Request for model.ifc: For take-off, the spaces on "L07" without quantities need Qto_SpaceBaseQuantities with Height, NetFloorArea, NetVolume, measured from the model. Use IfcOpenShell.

First a look at what the model holds.

```python
import ifcopenshell
import ifcopenshell.util.element
import ifcopenshell.util.unit

model = ifcopenshell.open("model.ifc")
print(model.schema)
for unit_type in ("LENGTHUNIT", "AREAUNIT", "VOLUMEUNIT"):
    print(unit_type, ifcopenshell.util.unit.calculate_unit_scale(model, unit_type))
storey = next(s for s in model.by_type("IfcBuildingStorey") if s.Name == "L07")
spaces = [e for e in ifcopenshell.util.element.get_decomposition(storey) if e.is_a("IfcSpace")]
for e in sorted(spaces, key=lambda e: e.id()):
    print(e.id(), e.is_a(), e.Name, list(ifcopenshell.util.element.get_psets(e, qtos_only=True)), sep=" | ")
```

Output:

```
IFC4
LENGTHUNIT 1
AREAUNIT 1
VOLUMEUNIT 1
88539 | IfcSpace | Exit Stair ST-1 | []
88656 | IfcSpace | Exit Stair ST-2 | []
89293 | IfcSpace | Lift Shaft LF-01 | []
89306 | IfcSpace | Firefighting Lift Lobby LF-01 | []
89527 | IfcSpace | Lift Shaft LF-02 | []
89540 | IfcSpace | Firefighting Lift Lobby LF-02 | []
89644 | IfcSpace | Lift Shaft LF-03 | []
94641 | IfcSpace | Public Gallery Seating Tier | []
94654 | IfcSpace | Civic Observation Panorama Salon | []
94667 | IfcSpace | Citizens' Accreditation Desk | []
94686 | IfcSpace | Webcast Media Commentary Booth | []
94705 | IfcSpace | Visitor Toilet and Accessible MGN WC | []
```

```python
import ifcopenshell
import ifcopenshell.api.pset
import ifcopenshell.geom
import ifcopenshell.util.element
import ifcopenshell.util.shape
import ifcopenshell.util.unit

model = ifcopenshell.open("model.ifc")
unit_scale = ifcopenshell.util.unit.calculate_unit_scale(model)
area_scale = ifcopenshell.util.unit.calculate_unit_scale(model, "AREAUNIT")
volume_scale = ifcopenshell.util.unit.calculate_unit_scale(model, "VOLUMEUNIT")
settings = ifcopenshell.geom.settings()

storey = next(s for s in model.by_type("IfcBuildingStorey") if s.Name == "L07")
spaces = [e for e in ifcopenshell.util.element.get_decomposition(storey) if e.is_a("IfcSpace")]

for e in sorted(spaces, key=lambda e: e.id()):
    if ifcopenshell.util.element.get_psets(e, qtos_only=True, should_inherit=False):
        continue
    # Geometry comes back in metres, in the element's own axes.
    shape = ifcopenshell.geom.create_shape(settings, e)
    values = {
        "Height": ifcopenshell.util.shape.get_z(shape.geometry) / unit_scale,
        "NetFloorArea": ifcopenshell.util.shape.get_footprint_area(shape.geometry) / area_scale,
        "NetVolume": ifcopenshell.util.shape.get_volume(shape.geometry) / volume_scale,
    }
    qto = ifcopenshell.api.pset.add_qto(model, product=e, name="Qto_SpaceBaseQuantities")
    ifcopenshell.api.pset.edit_qto(model, qto=qto, properties=values)
    print(e.id(), {k: round(v, 3) for k, v in values.items()})

model.write("model_updated.ifc")
```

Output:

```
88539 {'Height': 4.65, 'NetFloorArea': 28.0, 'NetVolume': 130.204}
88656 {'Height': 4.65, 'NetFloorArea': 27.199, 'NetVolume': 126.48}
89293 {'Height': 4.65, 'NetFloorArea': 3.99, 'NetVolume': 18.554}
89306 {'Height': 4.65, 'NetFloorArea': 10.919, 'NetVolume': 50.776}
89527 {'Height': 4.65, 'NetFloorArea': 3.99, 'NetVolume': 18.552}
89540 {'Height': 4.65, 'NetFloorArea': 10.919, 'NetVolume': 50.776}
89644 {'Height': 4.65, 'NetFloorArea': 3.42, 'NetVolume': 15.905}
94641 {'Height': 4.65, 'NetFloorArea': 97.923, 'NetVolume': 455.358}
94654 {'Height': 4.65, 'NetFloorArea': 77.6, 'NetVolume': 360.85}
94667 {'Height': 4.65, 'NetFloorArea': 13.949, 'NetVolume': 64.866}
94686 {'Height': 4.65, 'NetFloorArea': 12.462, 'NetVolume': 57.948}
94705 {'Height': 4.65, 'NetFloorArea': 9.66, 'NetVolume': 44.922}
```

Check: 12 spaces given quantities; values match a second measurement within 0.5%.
